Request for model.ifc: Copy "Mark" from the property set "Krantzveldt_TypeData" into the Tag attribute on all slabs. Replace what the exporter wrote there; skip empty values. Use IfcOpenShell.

First a look at what the model holds.

```python
import ifcopenshell
import ifcopenshell.util.element

model = ifcopenshell.open("model.ifc")
print(model.schema)
slabs = model.by_type("IfcSlab")
print(len(slabs), "slabs")
for e in slabs[:8]:
    source = ifcopenshell.util.element.get_pset(e, "Krantzveldt_TypeData", "Mark")
    target = e.Tag
    print(e.id(), repr(source), repr(target), sep=" | ")
```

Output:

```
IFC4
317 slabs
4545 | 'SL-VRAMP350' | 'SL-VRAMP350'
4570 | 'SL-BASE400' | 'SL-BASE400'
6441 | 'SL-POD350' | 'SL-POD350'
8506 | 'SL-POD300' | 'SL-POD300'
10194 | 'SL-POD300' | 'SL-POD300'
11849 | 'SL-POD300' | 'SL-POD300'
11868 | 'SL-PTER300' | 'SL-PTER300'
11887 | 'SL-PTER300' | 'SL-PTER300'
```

```python
import ifcopenshell
import ifcopenshell.util.element

model = ifcopenshell.open("model.ifc")

count = 0
for e in model.by_type("IfcSlab"):
    value = ifcopenshell.util.element.get_pset(e, "Krantzveldt_TypeData", "Mark")
    current = e.Tag
    if not value or not value.strip() or current == value:
        continue
    e.Tag = value
    count += 1

print(count, "slabs updated")

model.write("model_edited.ifc")
```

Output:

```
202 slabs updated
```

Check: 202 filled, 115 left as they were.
